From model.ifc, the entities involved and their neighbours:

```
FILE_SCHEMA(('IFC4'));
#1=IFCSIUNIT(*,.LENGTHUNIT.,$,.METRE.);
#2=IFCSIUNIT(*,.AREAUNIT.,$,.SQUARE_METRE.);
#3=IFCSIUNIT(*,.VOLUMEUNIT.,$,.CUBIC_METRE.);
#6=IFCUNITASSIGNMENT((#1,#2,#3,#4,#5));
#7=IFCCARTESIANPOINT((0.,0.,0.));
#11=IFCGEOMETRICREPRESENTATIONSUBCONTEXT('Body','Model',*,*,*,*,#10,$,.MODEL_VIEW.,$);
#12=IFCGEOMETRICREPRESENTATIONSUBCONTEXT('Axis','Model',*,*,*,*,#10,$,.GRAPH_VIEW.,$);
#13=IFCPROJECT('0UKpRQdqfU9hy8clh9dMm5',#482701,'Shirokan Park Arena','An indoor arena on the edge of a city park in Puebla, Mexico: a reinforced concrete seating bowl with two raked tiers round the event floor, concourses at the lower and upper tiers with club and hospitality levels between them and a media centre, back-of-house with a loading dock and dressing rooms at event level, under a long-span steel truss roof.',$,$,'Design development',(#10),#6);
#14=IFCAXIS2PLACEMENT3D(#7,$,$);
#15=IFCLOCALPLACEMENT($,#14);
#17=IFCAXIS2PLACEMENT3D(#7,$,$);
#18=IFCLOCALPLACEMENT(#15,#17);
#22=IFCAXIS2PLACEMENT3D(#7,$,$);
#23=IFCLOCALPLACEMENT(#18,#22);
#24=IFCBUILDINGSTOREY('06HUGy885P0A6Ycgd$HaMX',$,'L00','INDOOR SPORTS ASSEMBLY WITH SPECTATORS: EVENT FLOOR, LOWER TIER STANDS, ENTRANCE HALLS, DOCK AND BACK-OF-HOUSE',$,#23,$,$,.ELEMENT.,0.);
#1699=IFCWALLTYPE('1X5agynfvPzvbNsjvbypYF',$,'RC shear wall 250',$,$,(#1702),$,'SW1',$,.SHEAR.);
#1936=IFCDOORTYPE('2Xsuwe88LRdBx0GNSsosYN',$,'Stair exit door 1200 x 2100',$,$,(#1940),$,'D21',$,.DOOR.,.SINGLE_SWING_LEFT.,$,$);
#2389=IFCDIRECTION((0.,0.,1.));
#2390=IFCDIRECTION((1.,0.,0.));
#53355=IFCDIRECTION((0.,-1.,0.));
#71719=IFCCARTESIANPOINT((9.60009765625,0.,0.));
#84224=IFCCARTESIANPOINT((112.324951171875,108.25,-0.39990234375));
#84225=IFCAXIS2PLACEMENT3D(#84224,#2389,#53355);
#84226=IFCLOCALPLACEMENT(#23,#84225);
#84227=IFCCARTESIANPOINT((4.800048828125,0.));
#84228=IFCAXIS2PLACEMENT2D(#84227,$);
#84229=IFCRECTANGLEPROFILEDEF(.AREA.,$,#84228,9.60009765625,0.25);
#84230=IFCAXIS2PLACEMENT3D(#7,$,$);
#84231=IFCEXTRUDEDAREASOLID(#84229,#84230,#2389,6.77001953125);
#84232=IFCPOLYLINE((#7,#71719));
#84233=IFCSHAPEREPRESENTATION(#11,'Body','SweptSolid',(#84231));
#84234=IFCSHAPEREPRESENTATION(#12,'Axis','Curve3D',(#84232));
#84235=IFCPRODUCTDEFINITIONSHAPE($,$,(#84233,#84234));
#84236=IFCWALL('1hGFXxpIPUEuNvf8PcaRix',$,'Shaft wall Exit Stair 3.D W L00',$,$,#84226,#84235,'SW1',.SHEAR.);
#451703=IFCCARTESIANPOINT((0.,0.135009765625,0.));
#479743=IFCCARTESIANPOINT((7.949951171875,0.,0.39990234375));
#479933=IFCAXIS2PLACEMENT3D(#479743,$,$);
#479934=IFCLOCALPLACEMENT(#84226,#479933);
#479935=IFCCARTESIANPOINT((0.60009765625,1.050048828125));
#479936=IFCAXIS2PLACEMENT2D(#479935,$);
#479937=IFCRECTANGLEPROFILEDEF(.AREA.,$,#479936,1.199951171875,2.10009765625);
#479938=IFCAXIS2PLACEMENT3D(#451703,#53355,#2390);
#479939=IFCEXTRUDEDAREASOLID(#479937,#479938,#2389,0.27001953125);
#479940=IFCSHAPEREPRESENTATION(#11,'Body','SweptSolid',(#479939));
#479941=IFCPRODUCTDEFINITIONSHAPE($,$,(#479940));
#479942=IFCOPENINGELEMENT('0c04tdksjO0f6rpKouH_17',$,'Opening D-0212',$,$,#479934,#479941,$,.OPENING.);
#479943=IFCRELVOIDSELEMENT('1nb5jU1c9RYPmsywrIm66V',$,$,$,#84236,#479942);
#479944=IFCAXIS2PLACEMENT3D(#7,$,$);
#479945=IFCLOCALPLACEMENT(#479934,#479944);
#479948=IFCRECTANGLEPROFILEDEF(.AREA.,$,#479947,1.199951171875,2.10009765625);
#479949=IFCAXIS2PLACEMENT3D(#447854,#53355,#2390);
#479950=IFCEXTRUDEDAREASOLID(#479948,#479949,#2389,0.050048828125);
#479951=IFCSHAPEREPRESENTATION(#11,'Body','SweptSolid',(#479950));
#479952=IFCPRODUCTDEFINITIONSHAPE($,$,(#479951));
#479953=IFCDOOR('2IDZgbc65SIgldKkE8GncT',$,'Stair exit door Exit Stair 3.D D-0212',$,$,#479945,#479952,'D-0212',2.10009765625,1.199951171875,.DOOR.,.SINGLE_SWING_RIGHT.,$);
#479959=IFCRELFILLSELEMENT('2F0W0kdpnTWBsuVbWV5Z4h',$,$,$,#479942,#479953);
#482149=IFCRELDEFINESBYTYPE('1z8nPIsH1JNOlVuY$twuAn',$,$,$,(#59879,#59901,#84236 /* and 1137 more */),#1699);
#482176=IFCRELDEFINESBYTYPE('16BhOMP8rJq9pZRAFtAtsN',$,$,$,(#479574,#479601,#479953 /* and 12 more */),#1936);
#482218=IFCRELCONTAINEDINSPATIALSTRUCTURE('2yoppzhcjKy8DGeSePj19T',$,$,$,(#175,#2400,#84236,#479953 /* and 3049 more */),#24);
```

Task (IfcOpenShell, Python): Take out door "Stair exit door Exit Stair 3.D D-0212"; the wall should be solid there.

```python
import ifcopenshell
import ifcopenshell.api.feature
import ifcopenshell.api.root
import ifcopenshell.geom
import ifcopenshell.util.shape

model = ifcopenshell.open("model.ifc")
settings = ifcopenshell.geom.settings()


def volume(element):
    """Net volume in cubic metres, openings subtracted."""
    shape = ifcopenshell.geom.create_shape(settings, element)
    return ifcopenshell.util.shape.get_volume(shape.geometry)


door = model.by_id(479953)
opening = door.FillsVoids[0].RelatingOpeningElement
wall = opening.VoidsElements[0].RelatingBuildingElement
before = volume(wall)

ifcopenshell.api.root.remove_product(model, product=door)
ifcopenshell.api.feature.remove_feature(model, feature=opening)

after = volume(wall)

print(f"wall volume {before:.3f} -> {after:.3f} m3")

model.write("model-out.ifc")
```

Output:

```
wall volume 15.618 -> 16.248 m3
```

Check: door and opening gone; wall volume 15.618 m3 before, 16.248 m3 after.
